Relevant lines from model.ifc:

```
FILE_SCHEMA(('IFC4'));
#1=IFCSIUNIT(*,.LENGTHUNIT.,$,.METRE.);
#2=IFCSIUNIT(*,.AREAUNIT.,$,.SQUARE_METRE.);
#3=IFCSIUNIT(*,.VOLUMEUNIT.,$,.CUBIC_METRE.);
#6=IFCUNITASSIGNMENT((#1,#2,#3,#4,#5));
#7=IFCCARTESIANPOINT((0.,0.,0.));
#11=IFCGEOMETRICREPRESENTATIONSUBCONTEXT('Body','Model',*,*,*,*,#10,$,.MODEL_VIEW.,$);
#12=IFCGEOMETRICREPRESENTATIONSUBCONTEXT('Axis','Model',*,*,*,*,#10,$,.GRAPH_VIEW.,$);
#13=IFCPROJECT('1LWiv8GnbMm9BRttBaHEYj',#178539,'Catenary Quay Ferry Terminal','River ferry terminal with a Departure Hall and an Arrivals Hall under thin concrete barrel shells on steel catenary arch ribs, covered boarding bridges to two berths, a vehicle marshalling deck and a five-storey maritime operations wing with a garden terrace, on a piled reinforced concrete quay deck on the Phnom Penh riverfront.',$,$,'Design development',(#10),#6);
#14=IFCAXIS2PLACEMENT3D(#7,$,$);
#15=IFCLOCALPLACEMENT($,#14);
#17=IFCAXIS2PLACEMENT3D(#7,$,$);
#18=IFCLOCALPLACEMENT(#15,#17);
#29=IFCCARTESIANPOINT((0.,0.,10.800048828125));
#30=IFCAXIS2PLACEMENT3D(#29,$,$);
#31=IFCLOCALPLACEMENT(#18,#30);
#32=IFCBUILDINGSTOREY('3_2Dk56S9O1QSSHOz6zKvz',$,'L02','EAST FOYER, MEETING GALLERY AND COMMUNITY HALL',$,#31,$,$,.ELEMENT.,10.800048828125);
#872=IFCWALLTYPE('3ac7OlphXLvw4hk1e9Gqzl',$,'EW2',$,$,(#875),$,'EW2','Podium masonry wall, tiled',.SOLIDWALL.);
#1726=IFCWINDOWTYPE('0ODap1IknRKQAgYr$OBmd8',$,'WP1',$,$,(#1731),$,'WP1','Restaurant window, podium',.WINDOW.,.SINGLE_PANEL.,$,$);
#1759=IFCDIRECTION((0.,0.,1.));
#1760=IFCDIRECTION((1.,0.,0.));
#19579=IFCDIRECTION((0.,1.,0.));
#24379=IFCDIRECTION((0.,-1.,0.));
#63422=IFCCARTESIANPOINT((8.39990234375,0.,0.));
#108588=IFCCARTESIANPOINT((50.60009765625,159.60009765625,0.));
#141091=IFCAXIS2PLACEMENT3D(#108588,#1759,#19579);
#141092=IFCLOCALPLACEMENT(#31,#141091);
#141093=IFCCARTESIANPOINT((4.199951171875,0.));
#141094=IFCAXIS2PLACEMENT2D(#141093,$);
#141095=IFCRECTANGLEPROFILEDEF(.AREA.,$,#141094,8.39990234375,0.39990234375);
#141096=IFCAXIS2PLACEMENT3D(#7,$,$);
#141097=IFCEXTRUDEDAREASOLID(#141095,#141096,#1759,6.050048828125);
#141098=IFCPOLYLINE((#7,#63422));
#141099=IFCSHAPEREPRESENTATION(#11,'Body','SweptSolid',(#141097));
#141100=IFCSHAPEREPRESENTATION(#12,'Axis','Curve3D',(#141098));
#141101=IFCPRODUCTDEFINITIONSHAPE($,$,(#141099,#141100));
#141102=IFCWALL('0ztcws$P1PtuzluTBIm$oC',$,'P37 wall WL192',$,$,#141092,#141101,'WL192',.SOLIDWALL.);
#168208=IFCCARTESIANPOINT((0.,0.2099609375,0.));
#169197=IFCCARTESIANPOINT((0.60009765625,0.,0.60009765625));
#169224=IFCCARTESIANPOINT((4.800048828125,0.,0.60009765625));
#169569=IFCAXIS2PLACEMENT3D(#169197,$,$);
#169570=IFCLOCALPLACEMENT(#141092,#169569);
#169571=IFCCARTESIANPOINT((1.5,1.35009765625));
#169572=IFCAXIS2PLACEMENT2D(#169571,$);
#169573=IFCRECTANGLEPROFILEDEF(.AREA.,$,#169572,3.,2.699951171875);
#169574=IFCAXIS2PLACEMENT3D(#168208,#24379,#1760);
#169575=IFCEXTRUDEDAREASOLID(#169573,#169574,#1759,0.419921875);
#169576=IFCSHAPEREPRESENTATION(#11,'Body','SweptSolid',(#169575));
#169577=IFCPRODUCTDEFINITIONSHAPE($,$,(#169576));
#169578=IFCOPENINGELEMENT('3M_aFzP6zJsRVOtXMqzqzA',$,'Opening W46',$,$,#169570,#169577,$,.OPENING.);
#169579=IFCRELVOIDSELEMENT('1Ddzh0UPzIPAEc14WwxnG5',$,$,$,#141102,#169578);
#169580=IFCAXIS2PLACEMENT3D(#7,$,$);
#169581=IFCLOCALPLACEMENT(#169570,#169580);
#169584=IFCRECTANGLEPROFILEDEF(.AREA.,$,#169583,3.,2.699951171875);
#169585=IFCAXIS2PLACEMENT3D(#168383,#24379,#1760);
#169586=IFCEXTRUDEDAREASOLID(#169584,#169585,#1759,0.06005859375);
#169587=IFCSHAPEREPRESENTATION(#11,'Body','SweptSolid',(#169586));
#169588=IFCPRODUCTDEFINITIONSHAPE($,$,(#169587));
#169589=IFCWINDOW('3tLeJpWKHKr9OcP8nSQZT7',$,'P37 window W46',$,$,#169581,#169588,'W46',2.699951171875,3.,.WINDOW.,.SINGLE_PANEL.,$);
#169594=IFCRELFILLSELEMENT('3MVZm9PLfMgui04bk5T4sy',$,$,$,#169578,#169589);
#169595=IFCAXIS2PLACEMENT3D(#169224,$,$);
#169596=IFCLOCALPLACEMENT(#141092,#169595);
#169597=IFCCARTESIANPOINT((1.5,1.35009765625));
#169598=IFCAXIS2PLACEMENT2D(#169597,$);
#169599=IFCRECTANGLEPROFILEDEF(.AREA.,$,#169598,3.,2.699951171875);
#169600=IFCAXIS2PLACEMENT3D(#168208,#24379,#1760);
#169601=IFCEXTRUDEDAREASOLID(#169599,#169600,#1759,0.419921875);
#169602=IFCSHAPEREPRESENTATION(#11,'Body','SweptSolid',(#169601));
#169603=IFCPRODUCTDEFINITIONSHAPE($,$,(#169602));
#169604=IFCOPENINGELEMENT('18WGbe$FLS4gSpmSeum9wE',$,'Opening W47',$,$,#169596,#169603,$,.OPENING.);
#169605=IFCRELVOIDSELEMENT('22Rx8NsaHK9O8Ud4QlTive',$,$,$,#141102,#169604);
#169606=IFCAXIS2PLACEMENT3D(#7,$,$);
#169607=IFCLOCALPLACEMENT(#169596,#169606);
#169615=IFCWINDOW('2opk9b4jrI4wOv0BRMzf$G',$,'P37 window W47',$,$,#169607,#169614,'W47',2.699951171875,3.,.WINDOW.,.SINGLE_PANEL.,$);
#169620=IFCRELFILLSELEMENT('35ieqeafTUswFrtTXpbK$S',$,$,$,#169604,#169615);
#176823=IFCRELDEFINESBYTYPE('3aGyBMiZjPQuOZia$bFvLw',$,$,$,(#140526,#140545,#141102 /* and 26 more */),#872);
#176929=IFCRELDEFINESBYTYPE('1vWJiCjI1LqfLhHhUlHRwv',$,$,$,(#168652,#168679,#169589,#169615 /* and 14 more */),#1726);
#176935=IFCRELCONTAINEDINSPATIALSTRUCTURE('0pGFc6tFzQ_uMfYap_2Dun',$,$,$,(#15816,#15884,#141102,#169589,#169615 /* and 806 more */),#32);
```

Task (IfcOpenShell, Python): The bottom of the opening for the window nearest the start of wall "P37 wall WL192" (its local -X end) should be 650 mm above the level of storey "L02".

```python
import numpy as np
import ifcopenshell
import ifcopenshell.api.geometry
import ifcopenshell.geom
import ifcopenshell.util.element
import ifcopenshell.util.placement
import ifcopenshell.util.shape
import ifcopenshell.util.unit

model = ifcopenshell.open("model.ifc")
unit_scale = ifcopenshell.util.unit.calculate_unit_scale(model)

window = model.by_guid("3tLeJpWKHKr9OcP8nSQZT7")
opening = window.FillsVoids[0].RelatingOpeningElement
storey = ifcopenshell.util.element.get_container(window, ifc_class="IfcBuildingStorey")
level = ifcopenshell.util.placement.get_local_placement(storey.ObjectPlacement)[2, 3]

# The opening's origin need not be at the sill, so measure its lowest point.
shape = ifcopenshell.geom.create_shape(ifcopenshell.geom.settings(), opening)
bottom = ifcopenshell.util.shape.get_shape_bottom_elevation(shape, shape.geometry) / unit_scale
dz = level + 0.65 - bottom

shift = np.array([0.0, 0.0, dz])
# The window is placed relative to its opening, so it follows when the opening moves.
matrix = ifcopenshell.util.placement.get_local_placement(opening.ObjectPlacement)
matrix[:3, 3] += shift
ifcopenshell.api.geometry.edit_object_placement(
    model, product=opening, matrix=matrix, is_si=False, should_transform_children=True
)

print(f"moved by {dz * unit_scale:+.3f} m")

model.write("model_v2.ifc")
```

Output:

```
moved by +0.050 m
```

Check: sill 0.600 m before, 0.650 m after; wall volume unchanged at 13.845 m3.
